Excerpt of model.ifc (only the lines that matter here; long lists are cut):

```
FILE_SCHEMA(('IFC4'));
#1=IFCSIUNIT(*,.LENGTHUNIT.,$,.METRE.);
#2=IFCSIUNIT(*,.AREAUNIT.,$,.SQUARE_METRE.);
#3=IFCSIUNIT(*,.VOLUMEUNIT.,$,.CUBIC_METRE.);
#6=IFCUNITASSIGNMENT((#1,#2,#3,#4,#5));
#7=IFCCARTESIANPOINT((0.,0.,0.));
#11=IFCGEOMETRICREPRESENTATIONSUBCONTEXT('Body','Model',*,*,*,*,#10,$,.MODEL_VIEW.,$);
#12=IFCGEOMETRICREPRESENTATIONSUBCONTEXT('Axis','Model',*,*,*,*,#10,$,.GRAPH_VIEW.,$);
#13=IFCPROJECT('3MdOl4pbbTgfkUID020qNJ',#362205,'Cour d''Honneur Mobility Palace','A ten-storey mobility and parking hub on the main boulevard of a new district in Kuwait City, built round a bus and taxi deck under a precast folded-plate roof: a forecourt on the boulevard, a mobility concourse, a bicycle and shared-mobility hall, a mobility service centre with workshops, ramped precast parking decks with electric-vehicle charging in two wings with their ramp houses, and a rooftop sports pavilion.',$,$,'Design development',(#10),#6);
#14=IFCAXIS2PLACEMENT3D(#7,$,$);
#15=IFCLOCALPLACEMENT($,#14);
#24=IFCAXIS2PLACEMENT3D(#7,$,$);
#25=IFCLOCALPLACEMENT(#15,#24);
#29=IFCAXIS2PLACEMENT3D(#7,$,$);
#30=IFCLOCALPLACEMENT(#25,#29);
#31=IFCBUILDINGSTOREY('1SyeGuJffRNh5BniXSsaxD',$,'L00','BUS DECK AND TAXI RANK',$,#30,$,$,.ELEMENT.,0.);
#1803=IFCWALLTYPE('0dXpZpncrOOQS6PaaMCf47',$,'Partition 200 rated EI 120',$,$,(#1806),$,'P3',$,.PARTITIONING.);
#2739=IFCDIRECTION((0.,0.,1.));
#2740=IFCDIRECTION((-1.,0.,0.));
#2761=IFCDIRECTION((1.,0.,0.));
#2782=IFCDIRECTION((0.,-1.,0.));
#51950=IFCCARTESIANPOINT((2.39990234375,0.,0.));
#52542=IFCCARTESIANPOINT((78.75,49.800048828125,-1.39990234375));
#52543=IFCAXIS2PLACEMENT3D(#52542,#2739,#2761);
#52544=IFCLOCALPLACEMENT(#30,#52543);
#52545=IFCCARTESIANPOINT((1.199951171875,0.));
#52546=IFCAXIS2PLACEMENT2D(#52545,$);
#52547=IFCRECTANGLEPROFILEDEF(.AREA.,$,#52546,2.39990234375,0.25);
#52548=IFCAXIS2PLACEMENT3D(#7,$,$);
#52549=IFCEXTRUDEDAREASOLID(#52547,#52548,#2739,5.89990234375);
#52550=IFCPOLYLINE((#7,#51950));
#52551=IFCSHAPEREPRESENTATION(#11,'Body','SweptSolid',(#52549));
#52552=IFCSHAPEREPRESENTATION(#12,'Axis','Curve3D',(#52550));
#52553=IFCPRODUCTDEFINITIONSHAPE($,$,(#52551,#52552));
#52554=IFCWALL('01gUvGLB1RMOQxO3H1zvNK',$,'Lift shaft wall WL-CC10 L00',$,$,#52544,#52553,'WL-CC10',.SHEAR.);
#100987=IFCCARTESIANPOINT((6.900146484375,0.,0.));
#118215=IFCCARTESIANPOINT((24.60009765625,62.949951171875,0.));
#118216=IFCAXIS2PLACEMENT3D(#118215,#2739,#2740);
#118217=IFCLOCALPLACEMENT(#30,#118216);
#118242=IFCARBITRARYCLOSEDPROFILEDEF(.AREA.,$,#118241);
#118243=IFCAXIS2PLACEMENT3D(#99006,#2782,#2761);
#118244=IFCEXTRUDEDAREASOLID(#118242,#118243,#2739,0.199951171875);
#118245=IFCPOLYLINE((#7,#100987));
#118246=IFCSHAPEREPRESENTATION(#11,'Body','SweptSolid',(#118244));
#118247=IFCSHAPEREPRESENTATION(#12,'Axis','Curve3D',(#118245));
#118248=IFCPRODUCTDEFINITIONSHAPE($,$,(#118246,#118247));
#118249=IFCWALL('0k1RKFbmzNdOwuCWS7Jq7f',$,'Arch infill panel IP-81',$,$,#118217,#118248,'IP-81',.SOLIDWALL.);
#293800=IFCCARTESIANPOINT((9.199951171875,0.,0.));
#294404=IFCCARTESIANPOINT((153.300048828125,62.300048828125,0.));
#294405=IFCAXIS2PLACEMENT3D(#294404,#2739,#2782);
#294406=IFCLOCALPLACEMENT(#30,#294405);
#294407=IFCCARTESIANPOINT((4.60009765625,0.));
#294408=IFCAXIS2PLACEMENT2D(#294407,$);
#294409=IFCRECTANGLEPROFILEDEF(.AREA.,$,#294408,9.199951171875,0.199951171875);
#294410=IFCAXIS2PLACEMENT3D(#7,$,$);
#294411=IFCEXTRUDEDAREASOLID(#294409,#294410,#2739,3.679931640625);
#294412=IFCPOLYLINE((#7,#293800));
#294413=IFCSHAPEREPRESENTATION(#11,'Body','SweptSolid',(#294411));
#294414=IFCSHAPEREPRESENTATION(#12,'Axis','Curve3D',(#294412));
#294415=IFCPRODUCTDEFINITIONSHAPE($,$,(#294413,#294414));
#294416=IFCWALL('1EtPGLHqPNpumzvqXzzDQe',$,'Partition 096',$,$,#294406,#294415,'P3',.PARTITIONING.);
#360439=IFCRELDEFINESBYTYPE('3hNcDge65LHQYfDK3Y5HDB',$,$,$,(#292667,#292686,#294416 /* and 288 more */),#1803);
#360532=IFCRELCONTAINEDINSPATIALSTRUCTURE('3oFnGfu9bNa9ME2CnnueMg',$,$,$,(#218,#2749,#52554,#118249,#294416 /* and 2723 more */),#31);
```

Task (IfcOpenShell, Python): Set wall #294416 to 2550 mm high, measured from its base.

```python
import ifcopenshell
import ifcopenshell.geom
import ifcopenshell.util.representation
import ifcopenshell.util.shape
import ifcopenshell.util.unit

model = ifcopenshell.open("model.ifc")
unit_scale = ifcopenshell.util.unit.calculate_unit_scale(model)
settings = ifcopenshell.geom.settings()


def volume(element):
    """Net volume in cubic metres, openings subtracted."""
    shape = ifcopenshell.geom.create_shape(settings, element)
    return ifcopenshell.util.shape.get_volume(shape.geometry)


wall = model.by_guid("1EtPGLHqPNpumzvqXzzDQe")
before = volume(wall)

body = ifcopenshell.util.representation.get_representation(wall, "Model", "Body")
solid = body.Items[0]
old_height = solid.Depth
solid.Depth = 2.55 / unit_scale
after = volume(wall)

print(f"height {old_height:g} -> {solid.Depth:g}, volume {before:.3f} -> {after:.3f} m3")

model.write("model_updated.ifc")
```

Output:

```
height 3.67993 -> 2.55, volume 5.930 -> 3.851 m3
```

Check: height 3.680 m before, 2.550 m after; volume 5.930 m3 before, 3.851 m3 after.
